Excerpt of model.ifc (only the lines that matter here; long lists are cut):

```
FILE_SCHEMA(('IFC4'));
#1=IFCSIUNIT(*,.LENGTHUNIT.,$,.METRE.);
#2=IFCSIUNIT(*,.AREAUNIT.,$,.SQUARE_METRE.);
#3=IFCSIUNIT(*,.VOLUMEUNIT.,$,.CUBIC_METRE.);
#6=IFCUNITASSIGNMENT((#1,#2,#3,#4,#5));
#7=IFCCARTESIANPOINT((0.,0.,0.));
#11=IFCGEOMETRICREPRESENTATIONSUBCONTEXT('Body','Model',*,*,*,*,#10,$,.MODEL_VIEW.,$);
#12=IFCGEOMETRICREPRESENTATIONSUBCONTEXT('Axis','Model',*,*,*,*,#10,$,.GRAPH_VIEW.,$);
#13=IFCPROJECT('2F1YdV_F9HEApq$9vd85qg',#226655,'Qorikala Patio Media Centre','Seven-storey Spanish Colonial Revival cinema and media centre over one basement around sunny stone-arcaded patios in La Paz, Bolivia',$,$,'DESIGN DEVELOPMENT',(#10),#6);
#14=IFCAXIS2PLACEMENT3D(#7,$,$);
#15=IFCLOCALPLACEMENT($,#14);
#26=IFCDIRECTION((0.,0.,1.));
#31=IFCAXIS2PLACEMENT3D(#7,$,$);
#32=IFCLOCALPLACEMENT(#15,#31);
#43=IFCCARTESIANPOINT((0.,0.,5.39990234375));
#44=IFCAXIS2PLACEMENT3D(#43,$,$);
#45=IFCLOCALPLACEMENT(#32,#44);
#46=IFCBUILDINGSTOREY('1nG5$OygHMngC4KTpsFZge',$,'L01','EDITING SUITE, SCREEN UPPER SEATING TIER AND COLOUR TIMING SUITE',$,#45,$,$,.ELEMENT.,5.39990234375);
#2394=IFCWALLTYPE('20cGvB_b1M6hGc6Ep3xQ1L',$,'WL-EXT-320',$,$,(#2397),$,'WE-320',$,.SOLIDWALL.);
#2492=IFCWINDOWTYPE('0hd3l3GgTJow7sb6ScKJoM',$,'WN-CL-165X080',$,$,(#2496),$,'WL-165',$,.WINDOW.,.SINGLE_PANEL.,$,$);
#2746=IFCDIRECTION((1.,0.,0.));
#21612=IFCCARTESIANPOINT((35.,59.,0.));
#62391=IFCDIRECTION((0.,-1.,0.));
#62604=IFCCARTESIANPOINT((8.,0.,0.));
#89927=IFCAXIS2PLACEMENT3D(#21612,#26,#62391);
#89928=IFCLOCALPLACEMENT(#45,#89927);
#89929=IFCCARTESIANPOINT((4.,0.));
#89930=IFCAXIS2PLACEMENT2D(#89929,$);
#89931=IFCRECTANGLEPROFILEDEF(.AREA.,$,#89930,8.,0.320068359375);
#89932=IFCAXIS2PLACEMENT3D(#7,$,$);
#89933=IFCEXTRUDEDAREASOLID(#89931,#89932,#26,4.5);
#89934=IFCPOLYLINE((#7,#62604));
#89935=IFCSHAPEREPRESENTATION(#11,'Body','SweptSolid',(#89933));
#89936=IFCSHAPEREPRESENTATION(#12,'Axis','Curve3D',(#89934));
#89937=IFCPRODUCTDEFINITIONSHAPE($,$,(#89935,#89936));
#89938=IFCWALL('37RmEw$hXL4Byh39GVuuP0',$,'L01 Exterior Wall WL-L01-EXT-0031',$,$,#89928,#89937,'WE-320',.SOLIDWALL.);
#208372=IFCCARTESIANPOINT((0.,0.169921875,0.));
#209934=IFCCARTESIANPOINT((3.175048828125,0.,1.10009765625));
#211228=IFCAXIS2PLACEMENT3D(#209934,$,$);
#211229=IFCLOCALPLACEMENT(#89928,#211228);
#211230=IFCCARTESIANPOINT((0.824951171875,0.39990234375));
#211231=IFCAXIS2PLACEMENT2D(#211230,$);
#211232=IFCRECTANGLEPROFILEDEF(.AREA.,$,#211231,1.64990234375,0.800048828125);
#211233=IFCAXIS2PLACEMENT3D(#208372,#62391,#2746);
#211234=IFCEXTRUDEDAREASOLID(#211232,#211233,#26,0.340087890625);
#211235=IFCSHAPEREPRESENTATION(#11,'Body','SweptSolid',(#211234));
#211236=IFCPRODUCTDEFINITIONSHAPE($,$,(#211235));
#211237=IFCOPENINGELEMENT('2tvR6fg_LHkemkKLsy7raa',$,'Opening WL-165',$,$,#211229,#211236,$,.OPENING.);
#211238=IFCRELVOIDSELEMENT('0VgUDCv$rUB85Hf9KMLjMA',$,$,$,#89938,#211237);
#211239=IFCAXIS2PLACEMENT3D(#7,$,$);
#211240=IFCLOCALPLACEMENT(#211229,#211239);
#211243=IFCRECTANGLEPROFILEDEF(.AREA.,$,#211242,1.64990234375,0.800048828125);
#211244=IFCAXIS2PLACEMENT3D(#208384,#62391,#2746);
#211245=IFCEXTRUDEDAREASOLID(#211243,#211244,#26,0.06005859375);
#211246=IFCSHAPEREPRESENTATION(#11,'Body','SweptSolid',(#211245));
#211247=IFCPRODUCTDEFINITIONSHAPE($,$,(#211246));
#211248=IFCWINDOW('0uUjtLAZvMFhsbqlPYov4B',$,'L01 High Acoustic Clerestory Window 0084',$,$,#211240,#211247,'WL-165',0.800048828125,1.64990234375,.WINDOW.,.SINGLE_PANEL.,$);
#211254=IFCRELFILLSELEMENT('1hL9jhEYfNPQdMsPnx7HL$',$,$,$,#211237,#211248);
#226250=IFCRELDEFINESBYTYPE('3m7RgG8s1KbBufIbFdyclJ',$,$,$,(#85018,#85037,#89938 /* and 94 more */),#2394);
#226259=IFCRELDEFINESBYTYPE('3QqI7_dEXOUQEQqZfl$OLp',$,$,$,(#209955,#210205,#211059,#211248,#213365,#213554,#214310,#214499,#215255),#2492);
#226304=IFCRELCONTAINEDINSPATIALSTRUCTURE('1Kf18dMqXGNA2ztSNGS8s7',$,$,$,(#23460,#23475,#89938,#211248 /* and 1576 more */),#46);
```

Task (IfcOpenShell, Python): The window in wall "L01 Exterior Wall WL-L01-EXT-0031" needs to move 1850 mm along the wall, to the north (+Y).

```python
import ifcopenshell
import ifcopenshell.api.geometry
import ifcopenshell.util.placement

model = ifcopenshell.open("model.ifc")

window = model.by_guid("0uUjtLAZvMFhsbqlPYov4B")
opening = window.FillsVoids[0].RelatingOpeningElement
wall = opening.VoidsElements[0].RelatingBuildingElement

wall_matrix = ifcopenshell.util.placement.get_local_placement(wall.ObjectPlacement)
shift = wall_matrix[:3, 0] * -1.85
before = ifcopenshell.util.placement.get_local_placement(window.ObjectPlacement)[:3, 3].copy()

# The window is placed relative to its opening, so it follows when the opening moves.
matrix = ifcopenshell.util.placement.get_local_placement(opening.ObjectPlacement)
matrix[:3, 3] += shift
ifcopenshell.api.geometry.edit_object_placement(
    model, product=opening, matrix=matrix, is_si=False, should_transform_children=True
)

after = ifcopenshell.util.placement.get_local_placement(window.ObjectPlacement)[:3, 3]
print("window moved by", (after - before).round(3) + 0.0)

model.write("model_v2.ifc")
```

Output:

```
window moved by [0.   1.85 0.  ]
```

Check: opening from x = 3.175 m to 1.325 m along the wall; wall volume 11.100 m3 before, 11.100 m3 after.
